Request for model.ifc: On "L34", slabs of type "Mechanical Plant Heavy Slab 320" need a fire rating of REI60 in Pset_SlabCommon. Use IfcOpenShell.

First a look at what the model holds.

```python
import ifcopenshell
import ifcopenshell.util.element

model = ifcopenshell.open("model.ifc")
print(model.schema)
storey = next(s for s in model.by_type("IfcBuildingStorey") if s.Name == "L34")
slabs = [e for e in ifcopenshell.util.element.get_decomposition(storey) if e.is_a("IfcSlab")]
seen = {}
for e in slabs:
    element_type = ifcopenshell.util.element.get_type(e)
    key = (element_type.Name if element_type != e and element_type else None, ifcopenshell.util.element.get_pset(e, "Pset_SlabCommon", "FireRating"))
    seen[key] = seen.get(key, 0) + 1
for (name, value), count in sorted(seen.items(), key=str):
    print(count, "x", name, "|", value)
```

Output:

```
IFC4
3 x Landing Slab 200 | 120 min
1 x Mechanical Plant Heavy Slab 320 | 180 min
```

```python
import ifcopenshell
import ifcopenshell.api.pset
import ifcopenshell.util.element

model = ifcopenshell.open("model.ifc")

storey = next(s for s in model.by_type("IfcBuildingStorey") if s.Name == "L34")
slabs = [e for e in ifcopenshell.util.element.get_decomposition(storey) if e.is_a("IfcSlab")]

count = 0
for e in slabs:
    element_type = ifcopenshell.util.element.get_type(e)
    if element_type in (None, e) or element_type.Name != "Mechanical Plant Heavy Slab 320":
        continue
    # add_pset returns the element's existing set when there is one.
    pset = ifcopenshell.api.pset.add_pset(model, product=e, name="Pset_SlabCommon")
    ifcopenshell.api.pset.edit_pset(model, pset=pset, properties={"FireRating": "REI60"})
    count += 1

print(count, "slabs updated")

model.write("model_edited.ifc")
```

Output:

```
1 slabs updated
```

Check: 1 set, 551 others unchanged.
